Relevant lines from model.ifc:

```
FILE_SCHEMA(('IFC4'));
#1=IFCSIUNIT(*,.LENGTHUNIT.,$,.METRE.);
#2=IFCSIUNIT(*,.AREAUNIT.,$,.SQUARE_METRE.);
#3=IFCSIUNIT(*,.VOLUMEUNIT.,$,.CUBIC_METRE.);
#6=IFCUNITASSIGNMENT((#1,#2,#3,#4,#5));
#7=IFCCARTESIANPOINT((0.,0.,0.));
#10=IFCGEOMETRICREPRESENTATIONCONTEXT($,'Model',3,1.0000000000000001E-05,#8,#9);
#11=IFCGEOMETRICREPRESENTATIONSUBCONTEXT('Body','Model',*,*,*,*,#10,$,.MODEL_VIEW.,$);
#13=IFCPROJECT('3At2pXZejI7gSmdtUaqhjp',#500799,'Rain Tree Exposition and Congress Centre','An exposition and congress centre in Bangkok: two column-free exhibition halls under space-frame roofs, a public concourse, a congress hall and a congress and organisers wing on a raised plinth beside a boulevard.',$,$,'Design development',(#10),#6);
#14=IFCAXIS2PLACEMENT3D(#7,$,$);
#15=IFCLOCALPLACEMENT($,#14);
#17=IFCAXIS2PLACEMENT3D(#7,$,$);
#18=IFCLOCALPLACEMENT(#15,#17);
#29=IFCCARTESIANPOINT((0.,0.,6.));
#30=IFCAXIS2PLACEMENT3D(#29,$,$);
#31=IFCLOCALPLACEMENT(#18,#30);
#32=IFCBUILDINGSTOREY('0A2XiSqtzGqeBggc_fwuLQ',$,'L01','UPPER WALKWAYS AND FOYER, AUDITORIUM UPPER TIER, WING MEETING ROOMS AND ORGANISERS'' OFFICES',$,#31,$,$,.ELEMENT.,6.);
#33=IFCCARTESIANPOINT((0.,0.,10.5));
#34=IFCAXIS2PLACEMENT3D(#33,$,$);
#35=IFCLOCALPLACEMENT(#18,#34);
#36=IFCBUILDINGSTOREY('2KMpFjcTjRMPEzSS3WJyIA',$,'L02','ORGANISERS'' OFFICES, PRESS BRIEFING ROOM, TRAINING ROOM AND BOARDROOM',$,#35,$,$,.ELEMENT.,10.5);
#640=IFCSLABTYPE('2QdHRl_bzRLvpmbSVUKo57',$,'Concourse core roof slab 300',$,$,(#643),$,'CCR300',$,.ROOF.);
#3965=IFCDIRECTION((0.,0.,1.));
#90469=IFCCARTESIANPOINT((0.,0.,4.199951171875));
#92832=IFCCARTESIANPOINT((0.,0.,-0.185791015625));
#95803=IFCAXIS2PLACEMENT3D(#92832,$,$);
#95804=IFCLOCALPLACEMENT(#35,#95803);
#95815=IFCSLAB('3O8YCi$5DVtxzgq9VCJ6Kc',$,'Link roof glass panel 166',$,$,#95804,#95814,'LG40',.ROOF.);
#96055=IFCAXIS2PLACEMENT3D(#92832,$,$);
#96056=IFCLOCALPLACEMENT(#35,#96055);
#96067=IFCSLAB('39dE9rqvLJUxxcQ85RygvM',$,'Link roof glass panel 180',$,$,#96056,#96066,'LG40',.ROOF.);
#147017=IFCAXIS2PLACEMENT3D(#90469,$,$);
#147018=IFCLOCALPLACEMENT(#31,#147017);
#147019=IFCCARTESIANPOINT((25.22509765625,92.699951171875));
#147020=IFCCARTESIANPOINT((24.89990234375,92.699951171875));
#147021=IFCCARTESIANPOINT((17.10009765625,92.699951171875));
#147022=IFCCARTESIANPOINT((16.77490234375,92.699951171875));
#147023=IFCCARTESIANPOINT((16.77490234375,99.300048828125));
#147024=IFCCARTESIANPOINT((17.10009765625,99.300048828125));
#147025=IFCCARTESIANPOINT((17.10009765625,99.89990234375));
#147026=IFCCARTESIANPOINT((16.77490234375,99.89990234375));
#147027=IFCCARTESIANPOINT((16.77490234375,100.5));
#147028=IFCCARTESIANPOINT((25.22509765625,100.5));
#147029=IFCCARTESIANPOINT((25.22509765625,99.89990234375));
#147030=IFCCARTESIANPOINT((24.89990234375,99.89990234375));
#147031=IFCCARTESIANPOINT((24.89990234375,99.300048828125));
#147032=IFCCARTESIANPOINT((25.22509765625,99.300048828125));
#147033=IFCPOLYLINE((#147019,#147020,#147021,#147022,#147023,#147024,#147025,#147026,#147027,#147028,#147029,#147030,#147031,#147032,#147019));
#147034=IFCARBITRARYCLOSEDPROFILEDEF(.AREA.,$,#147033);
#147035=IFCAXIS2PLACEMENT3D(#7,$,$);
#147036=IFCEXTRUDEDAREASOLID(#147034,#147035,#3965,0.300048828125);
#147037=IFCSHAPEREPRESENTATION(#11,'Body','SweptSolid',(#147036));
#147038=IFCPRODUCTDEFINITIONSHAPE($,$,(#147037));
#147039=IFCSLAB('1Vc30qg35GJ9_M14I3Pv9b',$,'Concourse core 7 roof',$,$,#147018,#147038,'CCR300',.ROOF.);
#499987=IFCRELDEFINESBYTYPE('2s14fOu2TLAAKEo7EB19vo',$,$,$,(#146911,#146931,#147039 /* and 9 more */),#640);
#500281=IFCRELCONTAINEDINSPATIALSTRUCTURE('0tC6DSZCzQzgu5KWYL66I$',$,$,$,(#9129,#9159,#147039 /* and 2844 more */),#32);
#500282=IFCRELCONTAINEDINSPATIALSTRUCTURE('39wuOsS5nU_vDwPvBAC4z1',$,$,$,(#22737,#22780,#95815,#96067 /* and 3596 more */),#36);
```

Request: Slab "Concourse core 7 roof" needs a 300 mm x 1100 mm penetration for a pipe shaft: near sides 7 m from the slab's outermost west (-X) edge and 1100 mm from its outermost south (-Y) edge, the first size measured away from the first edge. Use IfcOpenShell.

```python
import numpy as np
import ifcopenshell
import ifcopenshell.api.feature
import ifcopenshell.api.geometry
import ifcopenshell.api.root
import ifcopenshell.geom
import ifcopenshell.util.placement
import ifcopenshell.util.representation
import ifcopenshell.util.shape
import ifcopenshell.util.unit

model = ifcopenshell.open("model.ifc")
unit_scale = ifcopenshell.util.unit.calculate_unit_scale(model)
settings = ifcopenshell.geom.settings()


def volume(element):
    """Net volume in cubic metres, openings subtracted."""
    shape = ifcopenshell.geom.create_shape(settings, element)
    return ifcopenshell.util.shape.get_volume(shape.geometry)


slab = model.by_guid("1Vc30qg35GJ9_M14I3Pv9b")
before = volume(slab)

# Extent in the slab's own axes, in metres. The edges named are its -X and -Y sides.
slab_shape = ifcopenshell.geom.create_shape(settings, slab)
vertices = ifcopenshell.util.shape.get_vertices(slab_shape.geometry)
x_min, y_min, bottom = vertices.min(axis=0)
top = vertices[:, 2].max()

opening = ifcopenshell.api.root.create_entity(model, ifc_class="IfcOpeningElement", name="Pipe shaft opening", predefined_type="OPENING")
context = ifcopenshell.util.representation.get_context(model, "Model", "Body", "MODEL_VIEW")
width, depth = 0.3, 1.1
outline = [(0.0, 0.0), (width, 0.0), (width, depth), (0.0, depth), (0.0, 0.0)]
# Overshoot both faces by 50 mm so the cut is clean.
shape = ifcopenshell.api.geometry.add_slab_representation(
    model, context=context, depth=top - bottom + 0.1, polyline=outline
)
ifcopenshell.api.geometry.assign_representation(model, product=opening, representation=shape)

matrix = ifcopenshell.util.placement.get_local_placement(slab.ObjectPlacement)
matrix[:, 3] = matrix @ np.append(np.array([x_min + 7, y_min + 1.1, bottom - 0.05]) / unit_scale, 1.0)
ifcopenshell.api.geometry.edit_object_placement(model, product=opening, matrix=matrix, is_si=False)
ifcopenshell.api.feature.add_feature(model, feature=opening, element=slab)

after = volume(slab)

print(f"slab volume {before:.3f} -> {after:.3f} m3")

model.write("model-out.ifc")
```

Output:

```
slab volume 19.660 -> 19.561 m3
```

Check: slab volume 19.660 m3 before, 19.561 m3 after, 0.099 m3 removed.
